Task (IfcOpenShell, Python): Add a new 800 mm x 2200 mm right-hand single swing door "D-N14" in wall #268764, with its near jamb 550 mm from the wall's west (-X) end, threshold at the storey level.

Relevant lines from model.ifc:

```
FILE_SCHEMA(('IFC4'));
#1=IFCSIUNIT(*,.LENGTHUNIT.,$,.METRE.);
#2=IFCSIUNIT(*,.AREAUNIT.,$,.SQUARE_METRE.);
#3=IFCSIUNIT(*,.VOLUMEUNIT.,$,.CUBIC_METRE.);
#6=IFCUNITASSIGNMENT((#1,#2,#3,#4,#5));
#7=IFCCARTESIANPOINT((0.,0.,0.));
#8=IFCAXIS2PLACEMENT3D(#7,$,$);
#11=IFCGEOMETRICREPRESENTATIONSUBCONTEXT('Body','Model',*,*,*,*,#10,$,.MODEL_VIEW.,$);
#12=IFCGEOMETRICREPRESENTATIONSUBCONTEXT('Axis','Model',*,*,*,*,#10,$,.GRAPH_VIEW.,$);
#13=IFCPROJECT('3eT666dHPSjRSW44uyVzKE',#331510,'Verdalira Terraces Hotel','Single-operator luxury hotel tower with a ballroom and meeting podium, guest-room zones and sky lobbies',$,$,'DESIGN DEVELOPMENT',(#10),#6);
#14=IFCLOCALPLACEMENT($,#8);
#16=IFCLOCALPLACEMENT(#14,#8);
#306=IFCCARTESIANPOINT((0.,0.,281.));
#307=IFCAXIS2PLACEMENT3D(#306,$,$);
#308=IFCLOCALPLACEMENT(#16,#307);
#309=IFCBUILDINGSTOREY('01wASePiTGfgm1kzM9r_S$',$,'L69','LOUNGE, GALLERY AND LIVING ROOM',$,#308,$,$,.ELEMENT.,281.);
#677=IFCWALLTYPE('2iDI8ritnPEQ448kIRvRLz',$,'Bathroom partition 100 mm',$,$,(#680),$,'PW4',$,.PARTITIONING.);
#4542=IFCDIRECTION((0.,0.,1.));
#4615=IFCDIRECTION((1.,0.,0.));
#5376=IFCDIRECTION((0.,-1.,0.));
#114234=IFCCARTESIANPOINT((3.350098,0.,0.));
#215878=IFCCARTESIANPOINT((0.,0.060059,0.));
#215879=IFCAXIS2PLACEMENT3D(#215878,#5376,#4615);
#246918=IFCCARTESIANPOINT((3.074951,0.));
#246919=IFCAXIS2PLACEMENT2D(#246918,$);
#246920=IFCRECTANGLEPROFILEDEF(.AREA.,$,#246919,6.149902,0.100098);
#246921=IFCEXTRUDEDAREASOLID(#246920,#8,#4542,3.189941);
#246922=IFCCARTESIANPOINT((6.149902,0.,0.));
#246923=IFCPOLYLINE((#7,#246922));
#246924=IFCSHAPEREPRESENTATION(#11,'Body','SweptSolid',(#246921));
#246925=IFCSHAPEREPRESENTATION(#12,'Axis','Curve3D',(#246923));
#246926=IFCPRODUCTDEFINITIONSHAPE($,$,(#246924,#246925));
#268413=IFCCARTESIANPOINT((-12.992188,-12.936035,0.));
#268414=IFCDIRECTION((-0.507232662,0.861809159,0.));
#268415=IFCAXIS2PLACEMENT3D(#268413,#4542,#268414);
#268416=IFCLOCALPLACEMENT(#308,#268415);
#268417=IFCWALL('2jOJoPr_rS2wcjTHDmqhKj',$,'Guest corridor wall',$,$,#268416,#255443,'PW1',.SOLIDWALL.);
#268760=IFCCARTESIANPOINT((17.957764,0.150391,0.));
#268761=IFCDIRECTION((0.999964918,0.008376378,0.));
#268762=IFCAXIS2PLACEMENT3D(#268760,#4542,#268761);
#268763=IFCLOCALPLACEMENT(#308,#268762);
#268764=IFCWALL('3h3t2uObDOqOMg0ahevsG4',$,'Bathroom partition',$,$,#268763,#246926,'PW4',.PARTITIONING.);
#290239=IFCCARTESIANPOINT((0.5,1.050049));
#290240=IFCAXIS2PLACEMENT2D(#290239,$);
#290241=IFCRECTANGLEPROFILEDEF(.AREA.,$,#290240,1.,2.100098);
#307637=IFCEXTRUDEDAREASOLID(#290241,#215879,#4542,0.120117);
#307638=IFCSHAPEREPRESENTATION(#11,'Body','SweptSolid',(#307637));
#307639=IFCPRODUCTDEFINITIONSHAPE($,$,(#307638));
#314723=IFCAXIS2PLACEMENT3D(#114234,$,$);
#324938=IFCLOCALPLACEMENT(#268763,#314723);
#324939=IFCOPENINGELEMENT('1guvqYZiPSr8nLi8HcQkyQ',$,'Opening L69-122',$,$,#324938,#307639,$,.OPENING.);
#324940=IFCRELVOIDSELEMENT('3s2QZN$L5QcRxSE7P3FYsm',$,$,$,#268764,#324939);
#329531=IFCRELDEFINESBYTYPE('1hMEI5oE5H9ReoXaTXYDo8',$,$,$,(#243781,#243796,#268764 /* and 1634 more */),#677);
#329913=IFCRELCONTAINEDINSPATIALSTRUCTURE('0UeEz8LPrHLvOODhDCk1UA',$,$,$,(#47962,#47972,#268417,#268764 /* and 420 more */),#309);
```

```python
import numpy as np
import ifcopenshell
import ifcopenshell.api.feature
import ifcopenshell.api.geometry
import ifcopenshell.api.root
import ifcopenshell.api.spatial
import ifcopenshell.geom
import ifcopenshell.util.element
import ifcopenshell.util.placement
import ifcopenshell.util.representation
import ifcopenshell.util.shape
import ifcopenshell.util.unit

model = ifcopenshell.open("model.ifc")
unit_scale = ifcopenshell.util.unit.calculate_unit_scale(model)
settings = ifcopenshell.geom.settings()


def volume(element):
    """Net volume in cubic metres, openings subtracted."""
    shape = ifcopenshell.geom.create_shape(settings, element)
    return ifcopenshell.util.shape.get_volume(shape.geometry)


wall = model.by_guid("3h3t2uObDOqOMg0ahevsG4")
storey = ifcopenshell.util.element.get_container(wall, ifc_class="IfcBuildingStorey")
context = ifcopenshell.util.representation.get_context(model, "Model", "Body", "MODEL_VIEW")
before = volume(wall)

width, height, from_end, sill = 0.8, 2.2, 0.55, 0.0  # metres

# The wall runs along its own X axis, and the end named is its -X end.
wall_shape = ifcopenshell.geom.create_shape(settings, wall)
x, y, z = ifcopenshell.util.shape.get_vertices(wall_shape.geometry).T
start = x.min() + from_end
face, thickness = float(y.min()), float(y.max() - y.min())
wall_matrix = ifcopenshell.util.placement.get_local_placement(wall.ObjectPlacement)
level = ifcopenshell.util.placement.get_local_placement(storey.ObjectPlacement)[2, 3]


def in_wall(x, y):
    """Placement at x, y metres in the wall's axes, at sill height."""
    matrix = wall_matrix.copy()
    matrix[:, 3] = wall_matrix @ np.array([x / unit_scale, y / unit_scale, 0.0, 1.0])
    matrix[2, 3] = level + sill / unit_scale
    return matrix


# Opening: a box that overshoots both wall faces by 50 mm.
opening = ifcopenshell.api.root.create_entity(model, ifc_class="IfcOpeningElement", predefined_type="OPENING")
box = ifcopenshell.api.geometry.add_wall_representation(
    model, context=context, length=width, height=height, thickness=thickness + 0.1
)
ifcopenshell.api.geometry.assign_representation(model, product=opening, representation=box)
ifcopenshell.api.geometry.edit_object_placement(model, product=opening, matrix=in_wall(start, face - 0.05), is_si=False)
ifcopenshell.api.feature.add_feature(model, feature=opening, element=wall)

door = ifcopenshell.api.root.create_entity(model, ifc_class="IfcDoor", name="D-N14", predefined_type="DOOR")
door.OverallWidth, door.OverallHeight = width / unit_scale, height / unit_scale
door.OperationType = "SINGLE_SWING_RIGHT"
body = ifcopenshell.api.geometry.add_door_representation(
    model,
    context=context,
    overall_width=door.OverallWidth,
    overall_height=door.OverallHeight,
    operation_type="SINGLE_SWING_RIGHT",
    lining_properties={"LiningDepth": thickness / unit_scale, "ThresholdDepth": thickness / unit_scale},
)
ifcopenshell.api.geometry.assign_representation(model, product=door, representation=body)
ifcopenshell.api.spatial.assign_container(model, products=[door], relating_structure=storey)
ifcopenshell.api.feature.add_filling(model, opening=opening, element=door)

# The lining spans the wall, so the door starts at the wall face.
ifcopenshell.api.geometry.edit_object_placement(model, product=door, matrix=in_wall(start, face), is_si=False)

after = volume(wall)

print(f"wall volume {before:.3f} -> {after:.3f} m3")

model.write("model_v2.ifc")
```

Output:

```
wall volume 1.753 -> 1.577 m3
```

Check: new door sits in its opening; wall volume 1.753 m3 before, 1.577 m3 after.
